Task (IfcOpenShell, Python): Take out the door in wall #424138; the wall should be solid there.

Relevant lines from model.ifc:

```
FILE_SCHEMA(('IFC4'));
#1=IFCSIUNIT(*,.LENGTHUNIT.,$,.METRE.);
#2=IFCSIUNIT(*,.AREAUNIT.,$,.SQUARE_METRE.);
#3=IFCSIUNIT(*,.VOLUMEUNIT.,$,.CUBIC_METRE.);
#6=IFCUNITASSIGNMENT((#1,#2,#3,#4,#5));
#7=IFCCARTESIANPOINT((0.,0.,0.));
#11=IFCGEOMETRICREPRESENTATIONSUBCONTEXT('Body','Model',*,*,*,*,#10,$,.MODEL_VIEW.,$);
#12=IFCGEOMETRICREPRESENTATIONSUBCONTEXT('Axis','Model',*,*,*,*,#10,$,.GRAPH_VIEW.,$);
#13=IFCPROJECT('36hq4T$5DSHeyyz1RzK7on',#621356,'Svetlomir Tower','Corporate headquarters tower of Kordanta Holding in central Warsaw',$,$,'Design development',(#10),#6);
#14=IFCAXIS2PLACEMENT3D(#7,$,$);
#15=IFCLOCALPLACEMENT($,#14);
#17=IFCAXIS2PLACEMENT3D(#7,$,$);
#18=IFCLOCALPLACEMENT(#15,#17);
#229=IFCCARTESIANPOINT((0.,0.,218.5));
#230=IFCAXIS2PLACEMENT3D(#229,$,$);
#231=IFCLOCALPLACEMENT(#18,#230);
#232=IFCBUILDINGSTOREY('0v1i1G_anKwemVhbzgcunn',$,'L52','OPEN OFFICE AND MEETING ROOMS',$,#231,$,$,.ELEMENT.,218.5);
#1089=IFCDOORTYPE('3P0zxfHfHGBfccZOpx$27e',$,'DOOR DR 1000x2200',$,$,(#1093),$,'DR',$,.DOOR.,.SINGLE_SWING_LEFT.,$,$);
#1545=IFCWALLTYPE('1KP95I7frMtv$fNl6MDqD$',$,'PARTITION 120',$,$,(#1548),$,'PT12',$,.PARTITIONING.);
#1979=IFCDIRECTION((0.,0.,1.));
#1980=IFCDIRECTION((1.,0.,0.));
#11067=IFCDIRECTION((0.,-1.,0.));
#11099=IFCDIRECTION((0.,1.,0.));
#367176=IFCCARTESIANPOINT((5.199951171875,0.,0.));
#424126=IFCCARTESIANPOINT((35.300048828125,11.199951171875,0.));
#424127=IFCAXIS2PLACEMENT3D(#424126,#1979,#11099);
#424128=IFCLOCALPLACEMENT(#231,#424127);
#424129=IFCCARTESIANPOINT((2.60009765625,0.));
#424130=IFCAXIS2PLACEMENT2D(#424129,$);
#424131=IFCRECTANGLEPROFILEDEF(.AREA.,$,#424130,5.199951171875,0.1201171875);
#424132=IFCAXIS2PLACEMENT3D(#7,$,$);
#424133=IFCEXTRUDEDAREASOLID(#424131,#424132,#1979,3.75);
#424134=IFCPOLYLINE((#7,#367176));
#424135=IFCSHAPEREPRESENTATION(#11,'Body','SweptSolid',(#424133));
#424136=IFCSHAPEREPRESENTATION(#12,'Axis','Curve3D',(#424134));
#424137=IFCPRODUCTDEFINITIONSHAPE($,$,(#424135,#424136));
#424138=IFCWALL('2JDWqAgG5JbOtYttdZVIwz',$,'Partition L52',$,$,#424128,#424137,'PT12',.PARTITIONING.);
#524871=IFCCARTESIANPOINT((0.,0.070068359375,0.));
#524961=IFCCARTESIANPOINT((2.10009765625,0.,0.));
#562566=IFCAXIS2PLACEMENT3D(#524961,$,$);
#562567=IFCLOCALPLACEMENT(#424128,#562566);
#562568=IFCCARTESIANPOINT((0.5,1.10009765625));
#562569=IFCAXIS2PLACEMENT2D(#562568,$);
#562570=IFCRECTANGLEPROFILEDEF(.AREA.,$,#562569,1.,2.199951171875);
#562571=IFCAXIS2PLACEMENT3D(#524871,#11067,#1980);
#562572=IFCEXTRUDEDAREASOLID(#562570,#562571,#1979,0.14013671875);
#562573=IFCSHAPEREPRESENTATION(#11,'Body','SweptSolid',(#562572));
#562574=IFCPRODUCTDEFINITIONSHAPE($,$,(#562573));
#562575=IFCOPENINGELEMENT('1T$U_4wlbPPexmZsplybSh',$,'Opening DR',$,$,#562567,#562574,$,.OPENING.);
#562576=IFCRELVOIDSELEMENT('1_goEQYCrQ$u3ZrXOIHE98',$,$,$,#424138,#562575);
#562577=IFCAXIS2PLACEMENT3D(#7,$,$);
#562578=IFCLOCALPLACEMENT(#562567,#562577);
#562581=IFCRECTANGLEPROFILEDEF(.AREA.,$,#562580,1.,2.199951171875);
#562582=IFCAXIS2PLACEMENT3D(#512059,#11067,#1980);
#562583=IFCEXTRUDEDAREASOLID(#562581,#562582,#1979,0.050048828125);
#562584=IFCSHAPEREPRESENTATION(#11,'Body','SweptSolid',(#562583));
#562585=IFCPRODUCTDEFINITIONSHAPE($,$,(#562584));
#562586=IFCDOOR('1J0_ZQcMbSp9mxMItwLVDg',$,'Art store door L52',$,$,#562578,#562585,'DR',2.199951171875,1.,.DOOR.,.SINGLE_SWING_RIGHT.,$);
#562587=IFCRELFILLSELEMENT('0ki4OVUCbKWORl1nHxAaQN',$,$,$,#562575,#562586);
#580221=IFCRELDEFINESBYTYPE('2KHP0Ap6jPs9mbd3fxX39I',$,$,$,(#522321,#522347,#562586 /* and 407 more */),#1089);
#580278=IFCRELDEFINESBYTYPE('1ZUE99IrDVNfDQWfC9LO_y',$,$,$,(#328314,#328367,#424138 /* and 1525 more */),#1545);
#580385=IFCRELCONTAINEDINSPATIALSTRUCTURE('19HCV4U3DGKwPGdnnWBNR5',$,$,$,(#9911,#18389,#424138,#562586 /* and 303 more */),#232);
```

```python
import ifcopenshell
import ifcopenshell.api.feature
import ifcopenshell.api.root
import ifcopenshell.geom
import ifcopenshell.util.shape

model = ifcopenshell.open("model.ifc")
settings = ifcopenshell.geom.settings()


def volume(element):
    """Net volume in cubic metres, openings subtracted."""
    shape = ifcopenshell.geom.create_shape(settings, element)
    return ifcopenshell.util.shape.get_volume(shape.geometry)


door = model.by_id(562586)
opening = door.FillsVoids[0].RelatingOpeningElement
wall = opening.VoidsElements[0].RelatingBuildingElement
before = volume(wall)

ifcopenshell.api.root.remove_product(model, product=door)
ifcopenshell.api.feature.remove_feature(model, feature=opening)

after = volume(wall)

print(f"wall volume {before:.3f} -> {after:.3f} m3")

model.write("model-out.ifc")
```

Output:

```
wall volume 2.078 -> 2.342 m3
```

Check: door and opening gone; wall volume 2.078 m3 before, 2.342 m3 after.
